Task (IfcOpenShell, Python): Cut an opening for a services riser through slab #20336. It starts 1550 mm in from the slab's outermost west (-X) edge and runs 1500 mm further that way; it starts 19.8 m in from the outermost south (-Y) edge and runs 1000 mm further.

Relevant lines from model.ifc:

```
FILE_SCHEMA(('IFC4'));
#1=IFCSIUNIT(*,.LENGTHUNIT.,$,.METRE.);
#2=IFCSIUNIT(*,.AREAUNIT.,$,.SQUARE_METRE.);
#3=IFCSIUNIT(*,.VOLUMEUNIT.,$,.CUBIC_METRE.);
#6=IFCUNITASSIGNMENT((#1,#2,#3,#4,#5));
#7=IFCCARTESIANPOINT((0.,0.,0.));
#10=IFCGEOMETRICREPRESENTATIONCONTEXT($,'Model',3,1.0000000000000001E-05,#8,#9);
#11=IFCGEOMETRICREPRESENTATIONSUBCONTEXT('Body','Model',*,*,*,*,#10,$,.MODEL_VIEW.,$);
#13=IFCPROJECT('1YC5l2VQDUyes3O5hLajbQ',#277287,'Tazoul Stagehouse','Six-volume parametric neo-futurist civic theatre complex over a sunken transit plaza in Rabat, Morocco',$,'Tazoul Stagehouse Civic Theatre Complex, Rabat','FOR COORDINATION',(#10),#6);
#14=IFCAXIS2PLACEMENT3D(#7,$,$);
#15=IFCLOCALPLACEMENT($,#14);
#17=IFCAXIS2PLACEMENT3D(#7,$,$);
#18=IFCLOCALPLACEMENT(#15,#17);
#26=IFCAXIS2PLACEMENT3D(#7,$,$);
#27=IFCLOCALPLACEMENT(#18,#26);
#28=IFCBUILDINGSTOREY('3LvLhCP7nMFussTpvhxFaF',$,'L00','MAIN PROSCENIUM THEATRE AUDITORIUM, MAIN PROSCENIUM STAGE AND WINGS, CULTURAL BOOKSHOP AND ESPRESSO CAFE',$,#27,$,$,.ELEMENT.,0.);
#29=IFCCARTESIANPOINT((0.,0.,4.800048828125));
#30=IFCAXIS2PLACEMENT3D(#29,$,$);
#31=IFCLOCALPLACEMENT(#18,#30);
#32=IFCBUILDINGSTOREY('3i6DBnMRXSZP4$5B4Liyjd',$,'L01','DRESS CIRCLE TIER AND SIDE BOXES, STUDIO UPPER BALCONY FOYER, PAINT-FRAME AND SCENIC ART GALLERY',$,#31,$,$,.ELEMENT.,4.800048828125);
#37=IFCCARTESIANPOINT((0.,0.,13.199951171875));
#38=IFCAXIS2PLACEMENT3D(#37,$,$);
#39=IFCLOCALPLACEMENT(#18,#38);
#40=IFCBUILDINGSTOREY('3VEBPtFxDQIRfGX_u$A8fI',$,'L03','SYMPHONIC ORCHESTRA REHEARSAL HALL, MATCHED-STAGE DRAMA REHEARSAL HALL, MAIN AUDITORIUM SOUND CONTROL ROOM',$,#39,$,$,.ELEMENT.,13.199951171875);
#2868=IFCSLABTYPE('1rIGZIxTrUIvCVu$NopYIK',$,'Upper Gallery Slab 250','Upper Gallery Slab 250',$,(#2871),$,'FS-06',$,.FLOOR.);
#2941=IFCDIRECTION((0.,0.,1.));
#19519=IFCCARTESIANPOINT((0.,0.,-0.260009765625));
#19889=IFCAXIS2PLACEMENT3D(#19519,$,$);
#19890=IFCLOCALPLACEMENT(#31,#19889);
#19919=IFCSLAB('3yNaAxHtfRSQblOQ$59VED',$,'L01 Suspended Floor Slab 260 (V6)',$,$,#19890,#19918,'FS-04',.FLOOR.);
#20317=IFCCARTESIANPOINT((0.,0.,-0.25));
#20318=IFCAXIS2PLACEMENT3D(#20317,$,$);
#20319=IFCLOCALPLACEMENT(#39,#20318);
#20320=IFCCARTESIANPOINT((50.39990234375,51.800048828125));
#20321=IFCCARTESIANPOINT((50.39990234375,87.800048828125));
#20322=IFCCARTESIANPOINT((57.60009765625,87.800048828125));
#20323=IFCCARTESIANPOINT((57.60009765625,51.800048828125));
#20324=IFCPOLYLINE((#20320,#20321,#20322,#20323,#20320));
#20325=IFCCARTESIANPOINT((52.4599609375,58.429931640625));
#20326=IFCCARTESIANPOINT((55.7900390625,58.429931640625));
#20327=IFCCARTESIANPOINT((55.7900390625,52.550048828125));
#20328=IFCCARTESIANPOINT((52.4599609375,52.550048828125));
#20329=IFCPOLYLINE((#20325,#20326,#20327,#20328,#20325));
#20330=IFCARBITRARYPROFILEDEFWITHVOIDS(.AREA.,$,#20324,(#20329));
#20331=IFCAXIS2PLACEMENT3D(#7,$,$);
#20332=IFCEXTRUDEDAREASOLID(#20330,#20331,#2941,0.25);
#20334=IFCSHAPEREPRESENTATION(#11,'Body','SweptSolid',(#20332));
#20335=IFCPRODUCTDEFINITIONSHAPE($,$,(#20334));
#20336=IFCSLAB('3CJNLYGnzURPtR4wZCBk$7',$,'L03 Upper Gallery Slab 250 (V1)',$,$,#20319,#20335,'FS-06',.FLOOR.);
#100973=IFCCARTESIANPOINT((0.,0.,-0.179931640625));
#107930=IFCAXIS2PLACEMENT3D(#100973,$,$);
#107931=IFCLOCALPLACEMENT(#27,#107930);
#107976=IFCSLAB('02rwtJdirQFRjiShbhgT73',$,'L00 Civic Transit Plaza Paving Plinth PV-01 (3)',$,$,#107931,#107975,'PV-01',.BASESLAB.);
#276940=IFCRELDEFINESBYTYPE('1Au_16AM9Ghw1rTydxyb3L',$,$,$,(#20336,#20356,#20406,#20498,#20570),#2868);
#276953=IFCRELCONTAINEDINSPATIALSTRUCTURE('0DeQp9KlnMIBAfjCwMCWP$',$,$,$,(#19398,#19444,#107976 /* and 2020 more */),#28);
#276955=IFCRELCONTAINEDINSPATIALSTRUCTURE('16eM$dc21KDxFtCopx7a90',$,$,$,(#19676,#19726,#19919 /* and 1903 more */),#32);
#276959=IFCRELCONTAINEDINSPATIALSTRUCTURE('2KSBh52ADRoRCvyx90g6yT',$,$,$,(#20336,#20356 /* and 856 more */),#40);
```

```python
import numpy as np
import ifcopenshell
import ifcopenshell.api.feature
import ifcopenshell.api.geometry
import ifcopenshell.api.root
import ifcopenshell.geom
import ifcopenshell.util.placement
import ifcopenshell.util.representation
import ifcopenshell.util.shape
import ifcopenshell.util.unit

model = ifcopenshell.open("model.ifc")
unit_scale = ifcopenshell.util.unit.calculate_unit_scale(model)
settings = ifcopenshell.geom.settings()


def volume(element):
    """Net volume in cubic metres, openings subtracted."""
    shape = ifcopenshell.geom.create_shape(settings, element)
    return ifcopenshell.util.shape.get_volume(shape.geometry)


slab = model.by_guid("3CJNLYGnzURPtR4wZCBk$7")
before = volume(slab)

# Extent in the slab's own axes, in metres. The edges named are its -X and -Y sides.
slab_shape = ifcopenshell.geom.create_shape(settings, slab)
vertices = ifcopenshell.util.shape.get_vertices(slab_shape.geometry)
x_min, y_min, bottom = vertices.min(axis=0)
top = vertices[:, 2].max()

opening = ifcopenshell.api.root.create_entity(model, ifc_class="IfcOpeningElement", name="Services riser opening", predefined_type="OPENING")
context = ifcopenshell.util.representation.get_context(model, "Model", "Body", "MODEL_VIEW")
width, depth = 1.5, 1
outline = [(0.0, 0.0), (width, 0.0), (width, depth), (0.0, depth), (0.0, 0.0)]
# Overshoot both faces by 50 mm so the cut is clean.
shape = ifcopenshell.api.geometry.add_slab_representation(
    model, context=context, depth=top - bottom + 0.1, polyline=outline
)
ifcopenshell.api.geometry.assign_representation(model, product=opening, representation=shape)

matrix = ifcopenshell.util.placement.get_local_placement(slab.ObjectPlacement)
matrix[:, 3] = matrix @ np.append(np.array([x_min + 1.55, y_min + 19.8, bottom - 0.05]) / unit_scale, 1.0)
ifcopenshell.api.geometry.edit_object_placement(model, product=opening, matrix=matrix, is_si=False)
ifcopenshell.api.feature.add_feature(model, feature=opening, element=slab)

after = volume(slab)

print(f"slab volume {before:.3f} -> {after:.3f} m3")

model.write("model_updated.ifc")
```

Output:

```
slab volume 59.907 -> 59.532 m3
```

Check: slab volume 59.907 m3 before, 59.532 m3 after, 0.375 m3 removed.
